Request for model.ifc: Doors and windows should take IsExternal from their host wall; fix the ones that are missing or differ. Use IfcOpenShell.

First a look at what the model holds.

```python
import ifcopenshell
import ifcopenshell.util.element

model = ifcopenshell.open("model.ifc")
print(model.schema)
seen = {}
for e in model.by_type("IfcDoor") + model.by_type("IfcWindow"):
    if not e.FillsVoids:
        continue
    host = e.FillsVoids[0].RelatingOpeningElement.VoidsElements[0].RelatingBuildingElement
    own = ifcopenshell.util.element.get_pset(e, f"Pset_{e.is_a()[3:].removesuffix('StandardCase')}Common", "IsExternal")
    wall = ifcopenshell.util.element.get_pset(host, "Pset_WallCommon", "IsExternal")
    seen[e.is_a(), own, wall] = seen.get((e.is_a(), own, wall), 0) + 1
for (cls, own, wall), count in sorted(seen.items(), key=str):
    print(count, cls, "IsExternal:", own, "| host wall:", wall)
```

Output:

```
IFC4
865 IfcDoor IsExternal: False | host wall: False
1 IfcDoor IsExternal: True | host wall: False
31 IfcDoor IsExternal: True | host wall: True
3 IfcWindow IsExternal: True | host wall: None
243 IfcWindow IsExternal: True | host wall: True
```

```python
import ifcopenshell
import ifcopenshell.api.pset
import ifcopenshell.util.element

model = ifcopenshell.open("model.ifc")

count = 0
for ifc_class, pset_name in (("IfcDoor", "Pset_DoorCommon"), ("IfcWindow", "Pset_WindowCommon")):
    for e in model.by_type(ifc_class):
        if not e.FillsVoids:
            continue
        host = e.FillsVoids[0].RelatingOpeningElement.VoidsElements[0].RelatingBuildingElement
        external = ifcopenshell.util.element.get_pset(host, "Pset_WallCommon", "IsExternal")
        if external is None or ifcopenshell.util.element.get_pset(e, pset_name, "IsExternal") == external:
            continue
        pset = ifcopenshell.api.pset.add_pset(model, product=e, name=pset_name)
        ifcopenshell.api.pset.edit_pset(model, pset=pset, properties={"IsExternal": external})
        count += 1

print(count, "updated")

model.write("model_edited.ifc")
```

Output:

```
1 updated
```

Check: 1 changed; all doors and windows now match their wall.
